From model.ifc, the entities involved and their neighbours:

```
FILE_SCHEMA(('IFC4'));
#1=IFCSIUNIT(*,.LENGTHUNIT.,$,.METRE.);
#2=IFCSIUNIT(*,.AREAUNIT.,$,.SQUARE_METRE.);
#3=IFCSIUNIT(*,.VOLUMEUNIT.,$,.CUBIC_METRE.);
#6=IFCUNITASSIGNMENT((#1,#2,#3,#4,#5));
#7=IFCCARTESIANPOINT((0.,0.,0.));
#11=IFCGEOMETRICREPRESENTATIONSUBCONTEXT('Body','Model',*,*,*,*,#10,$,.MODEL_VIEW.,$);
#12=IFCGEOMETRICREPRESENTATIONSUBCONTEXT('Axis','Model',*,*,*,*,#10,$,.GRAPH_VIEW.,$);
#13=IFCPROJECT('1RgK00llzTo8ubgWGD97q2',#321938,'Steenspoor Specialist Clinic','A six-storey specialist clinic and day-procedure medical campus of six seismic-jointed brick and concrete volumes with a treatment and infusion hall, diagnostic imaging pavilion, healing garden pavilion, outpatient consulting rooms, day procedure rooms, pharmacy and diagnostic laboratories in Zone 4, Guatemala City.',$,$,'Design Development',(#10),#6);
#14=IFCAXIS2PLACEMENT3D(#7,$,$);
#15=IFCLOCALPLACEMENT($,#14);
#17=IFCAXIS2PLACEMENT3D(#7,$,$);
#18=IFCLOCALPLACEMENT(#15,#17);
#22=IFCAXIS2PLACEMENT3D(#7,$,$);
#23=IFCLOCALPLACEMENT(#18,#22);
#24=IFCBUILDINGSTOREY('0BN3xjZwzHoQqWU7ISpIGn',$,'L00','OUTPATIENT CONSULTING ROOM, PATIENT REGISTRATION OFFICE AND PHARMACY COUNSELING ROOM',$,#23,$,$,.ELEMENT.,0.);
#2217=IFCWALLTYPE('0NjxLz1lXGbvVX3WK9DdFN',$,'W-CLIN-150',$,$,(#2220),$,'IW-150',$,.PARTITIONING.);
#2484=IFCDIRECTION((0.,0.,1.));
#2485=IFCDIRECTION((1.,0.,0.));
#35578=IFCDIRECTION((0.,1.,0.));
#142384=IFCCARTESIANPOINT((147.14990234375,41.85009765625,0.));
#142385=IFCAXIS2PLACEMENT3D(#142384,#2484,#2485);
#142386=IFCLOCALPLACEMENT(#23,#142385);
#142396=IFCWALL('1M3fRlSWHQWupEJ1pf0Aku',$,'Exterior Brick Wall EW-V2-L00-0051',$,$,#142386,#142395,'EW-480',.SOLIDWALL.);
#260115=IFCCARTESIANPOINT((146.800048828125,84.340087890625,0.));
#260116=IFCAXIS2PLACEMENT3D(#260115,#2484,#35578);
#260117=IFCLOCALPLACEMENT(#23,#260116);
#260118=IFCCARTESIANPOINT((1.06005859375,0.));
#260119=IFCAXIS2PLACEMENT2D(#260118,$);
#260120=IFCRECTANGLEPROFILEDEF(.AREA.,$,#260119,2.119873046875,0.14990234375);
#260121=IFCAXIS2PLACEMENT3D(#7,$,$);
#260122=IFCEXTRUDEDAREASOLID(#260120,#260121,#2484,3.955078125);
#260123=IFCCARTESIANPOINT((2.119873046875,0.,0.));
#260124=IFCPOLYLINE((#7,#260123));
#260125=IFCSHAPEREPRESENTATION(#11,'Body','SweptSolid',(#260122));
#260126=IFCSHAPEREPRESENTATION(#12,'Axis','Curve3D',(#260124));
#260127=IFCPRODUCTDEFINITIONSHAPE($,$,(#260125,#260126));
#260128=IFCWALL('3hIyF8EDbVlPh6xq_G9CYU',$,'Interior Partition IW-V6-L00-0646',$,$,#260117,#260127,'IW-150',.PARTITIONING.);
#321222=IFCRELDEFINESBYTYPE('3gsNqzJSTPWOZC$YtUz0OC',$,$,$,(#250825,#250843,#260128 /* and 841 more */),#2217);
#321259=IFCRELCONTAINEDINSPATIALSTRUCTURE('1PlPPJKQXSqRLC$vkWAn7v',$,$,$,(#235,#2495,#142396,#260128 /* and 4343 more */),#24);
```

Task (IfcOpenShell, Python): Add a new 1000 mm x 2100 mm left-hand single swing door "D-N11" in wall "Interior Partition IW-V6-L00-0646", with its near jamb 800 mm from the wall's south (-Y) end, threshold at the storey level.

```python
import numpy as np
import ifcopenshell
import ifcopenshell.api.feature
import ifcopenshell.api.geometry
import ifcopenshell.api.root
import ifcopenshell.api.spatial
import ifcopenshell.geom
import ifcopenshell.util.element
import ifcopenshell.util.placement
import ifcopenshell.util.representation
import ifcopenshell.util.shape
import ifcopenshell.util.unit

model = ifcopenshell.open("model.ifc")
unit_scale = ifcopenshell.util.unit.calculate_unit_scale(model)
settings = ifcopenshell.geom.settings()


def volume(element):
    """Net volume in cubic metres, openings subtracted."""
    shape = ifcopenshell.geom.create_shape(settings, element)
    return ifcopenshell.util.shape.get_volume(shape.geometry)


wall = model.by_id(260128)
storey = ifcopenshell.util.element.get_container(wall, ifc_class="IfcBuildingStorey")
context = ifcopenshell.util.representation.get_context(model, "Model", "Body", "MODEL_VIEW")
before = volume(wall)

width, height, from_end, sill = 1, 2.1, 0.8, 0.0  # metres

# The wall runs along its own X axis, and the end named is its -X end.
wall_shape = ifcopenshell.geom.create_shape(settings, wall)
x, y, z = ifcopenshell.util.shape.get_vertices(wall_shape.geometry).T
start = x.min() + from_end
face, thickness = float(y.min()), float(y.max() - y.min())
wall_matrix = ifcopenshell.util.placement.get_local_placement(wall.ObjectPlacement)
level = ifcopenshell.util.placement.get_local_placement(storey.ObjectPlacement)[2, 3]


def in_wall(x, y):
    """Placement at x, y metres in the wall's axes, at sill height."""
    matrix = wall_matrix.copy()
    matrix[:, 3] = wall_matrix @ np.array([x / unit_scale, y / unit_scale, 0.0, 1.0])
    matrix[2, 3] = level + sill / unit_scale
    return matrix


# Opening: a box that overshoots both wall faces by 50 mm.
opening = ifcopenshell.api.root.create_entity(model, ifc_class="IfcOpeningElement", predefined_type="OPENING")
box = ifcopenshell.api.geometry.add_wall_representation(
    model, context=context, length=width, height=height, thickness=thickness + 0.1
)
ifcopenshell.api.geometry.assign_representation(model, product=opening, representation=box)
ifcopenshell.api.geometry.edit_object_placement(model, product=opening, matrix=in_wall(start, face - 0.05), is_si=False)
ifcopenshell.api.feature.add_feature(model, feature=opening, element=wall)

door = ifcopenshell.api.root.create_entity(model, ifc_class="IfcDoor", name="D-N11", predefined_type="DOOR")
door.OverallWidth, door.OverallHeight = width / unit_scale, height / unit_scale
door.OperationType = "SINGLE_SWING_LEFT"
body = ifcopenshell.api.geometry.add_door_representation(
    model,
    context=context,
    overall_width=door.OverallWidth,
    overall_height=door.OverallHeight,
    operation_type="SINGLE_SWING_LEFT",
    lining_properties={"LiningDepth": thickness / unit_scale, "ThresholdDepth": thickness / unit_scale},
)
ifcopenshell.api.geometry.assign_representation(model, product=door, representation=body)
ifcopenshell.api.spatial.assign_container(model, products=[door], relating_structure=storey)
ifcopenshell.api.feature.add_filling(model, opening=opening, element=door)

# The lining spans the wall, so the door starts at the wall face.
ifcopenshell.api.geometry.edit_object_placement(model, product=door, matrix=in_wall(start, face), is_si=False)

after = volume(wall)

print(f"wall volume {before:.3f} -> {after:.3f} m3")

model.write("model_edited.ifc")
```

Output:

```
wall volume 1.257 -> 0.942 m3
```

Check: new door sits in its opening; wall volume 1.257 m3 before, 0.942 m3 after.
